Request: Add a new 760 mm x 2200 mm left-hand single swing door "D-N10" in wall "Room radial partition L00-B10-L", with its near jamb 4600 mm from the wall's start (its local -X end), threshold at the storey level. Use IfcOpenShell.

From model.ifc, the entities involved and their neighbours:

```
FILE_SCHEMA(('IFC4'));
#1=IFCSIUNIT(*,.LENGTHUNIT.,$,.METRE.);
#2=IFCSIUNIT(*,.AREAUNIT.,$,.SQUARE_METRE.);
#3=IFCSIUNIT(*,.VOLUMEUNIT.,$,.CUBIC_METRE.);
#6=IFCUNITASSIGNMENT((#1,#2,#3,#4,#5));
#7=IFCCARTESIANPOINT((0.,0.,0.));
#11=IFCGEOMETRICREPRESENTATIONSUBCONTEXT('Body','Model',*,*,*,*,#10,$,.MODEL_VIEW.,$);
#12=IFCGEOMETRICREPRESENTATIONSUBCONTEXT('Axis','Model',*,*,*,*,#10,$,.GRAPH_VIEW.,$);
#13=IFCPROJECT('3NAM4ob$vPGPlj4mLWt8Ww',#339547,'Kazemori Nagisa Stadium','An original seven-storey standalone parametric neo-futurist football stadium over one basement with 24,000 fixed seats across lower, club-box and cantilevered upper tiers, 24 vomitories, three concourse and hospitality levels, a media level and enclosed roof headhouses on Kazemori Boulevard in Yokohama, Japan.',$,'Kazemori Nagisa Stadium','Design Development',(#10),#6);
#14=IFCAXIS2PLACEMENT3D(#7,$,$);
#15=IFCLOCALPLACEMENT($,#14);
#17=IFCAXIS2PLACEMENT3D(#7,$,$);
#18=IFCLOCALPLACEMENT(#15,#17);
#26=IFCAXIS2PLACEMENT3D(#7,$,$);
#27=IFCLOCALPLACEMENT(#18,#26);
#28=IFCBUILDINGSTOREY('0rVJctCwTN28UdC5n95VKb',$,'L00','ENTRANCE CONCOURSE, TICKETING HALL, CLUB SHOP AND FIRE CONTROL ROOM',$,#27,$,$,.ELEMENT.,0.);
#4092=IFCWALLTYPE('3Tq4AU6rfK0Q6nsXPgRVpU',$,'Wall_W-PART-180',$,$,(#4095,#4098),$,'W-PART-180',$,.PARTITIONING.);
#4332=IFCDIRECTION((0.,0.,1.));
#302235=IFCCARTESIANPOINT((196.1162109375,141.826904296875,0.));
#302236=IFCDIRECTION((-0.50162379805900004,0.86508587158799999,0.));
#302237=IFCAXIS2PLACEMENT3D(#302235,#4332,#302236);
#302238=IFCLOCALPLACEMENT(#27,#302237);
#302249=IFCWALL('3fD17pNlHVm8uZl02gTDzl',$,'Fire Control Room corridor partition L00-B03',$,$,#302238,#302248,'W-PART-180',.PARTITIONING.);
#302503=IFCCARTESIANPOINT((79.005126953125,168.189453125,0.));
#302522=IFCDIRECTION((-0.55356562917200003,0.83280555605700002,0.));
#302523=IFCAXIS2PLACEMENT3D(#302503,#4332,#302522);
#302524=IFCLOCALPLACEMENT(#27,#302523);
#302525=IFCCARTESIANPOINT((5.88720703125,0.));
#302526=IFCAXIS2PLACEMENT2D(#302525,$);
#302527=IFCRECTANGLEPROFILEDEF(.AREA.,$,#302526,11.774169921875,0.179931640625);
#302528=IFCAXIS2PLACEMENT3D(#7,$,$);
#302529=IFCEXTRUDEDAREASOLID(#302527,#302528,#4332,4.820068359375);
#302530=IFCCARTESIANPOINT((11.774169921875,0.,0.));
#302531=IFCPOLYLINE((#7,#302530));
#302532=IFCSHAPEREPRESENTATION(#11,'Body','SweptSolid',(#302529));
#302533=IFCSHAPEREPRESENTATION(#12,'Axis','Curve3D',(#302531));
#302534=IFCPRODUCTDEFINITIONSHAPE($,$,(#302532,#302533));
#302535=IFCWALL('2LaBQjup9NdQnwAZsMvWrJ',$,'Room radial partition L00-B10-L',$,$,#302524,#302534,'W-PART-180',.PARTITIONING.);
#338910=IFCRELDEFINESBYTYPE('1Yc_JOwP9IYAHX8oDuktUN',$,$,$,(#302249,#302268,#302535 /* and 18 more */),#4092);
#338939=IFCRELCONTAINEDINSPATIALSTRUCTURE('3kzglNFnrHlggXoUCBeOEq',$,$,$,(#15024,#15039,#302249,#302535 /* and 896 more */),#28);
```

```python
import numpy as np
import ifcopenshell
import ifcopenshell.api.feature
import ifcopenshell.api.geometry
import ifcopenshell.api.root
import ifcopenshell.api.spatial
import ifcopenshell.geom
import ifcopenshell.util.element
import ifcopenshell.util.placement
import ifcopenshell.util.representation
import ifcopenshell.util.shape
import ifcopenshell.util.unit

model = ifcopenshell.open("model.ifc")
unit_scale = ifcopenshell.util.unit.calculate_unit_scale(model)
settings = ifcopenshell.geom.settings()


def volume(element):
    """Net volume in cubic metres, openings subtracted."""
    shape = ifcopenshell.geom.create_shape(settings, element)
    return ifcopenshell.util.shape.get_volume(shape.geometry)


wall = model.by_guid("2LaBQjup9NdQnwAZsMvWrJ")
storey = ifcopenshell.util.element.get_container(wall, ifc_class="IfcBuildingStorey")
context = ifcopenshell.util.representation.get_context(model, "Model", "Body", "MODEL_VIEW")
before = volume(wall)

width, height, from_end, sill = 0.76, 2.2, 4.6, 0.0  # metres

# The wall runs along its own X axis, and the end named is its -X end.
wall_shape = ifcopenshell.geom.create_shape(settings, wall)
x, y, z = ifcopenshell.util.shape.get_vertices(wall_shape.geometry).T
start = x.min() + from_end
face, thickness = float(y.min()), float(y.max() - y.min())
wall_matrix = ifcopenshell.util.placement.get_local_placement(wall.ObjectPlacement)
level = ifcopenshell.util.placement.get_local_placement(storey.ObjectPlacement)[2, 3]


def in_wall(x, y):
    """Placement at x, y metres in the wall's axes, at sill height."""
    matrix = wall_matrix.copy()
    matrix[:, 3] = wall_matrix @ np.array([x / unit_scale, y / unit_scale, 0.0, 1.0])
    matrix[2, 3] = level + sill / unit_scale
    return matrix


# Opening: a box that overshoots both wall faces by 50 mm.
opening = ifcopenshell.api.root.create_entity(model, ifc_class="IfcOpeningElement", predefined_type="OPENING")
box = ifcopenshell.api.geometry.add_wall_representation(
    model, context=context, length=width, height=height, thickness=thickness + 0.1
)
ifcopenshell.api.geometry.assign_representation(model, product=opening, representation=box)
ifcopenshell.api.geometry.edit_object_placement(model, product=opening, matrix=in_wall(start, face - 0.05), is_si=False)
ifcopenshell.api.feature.add_feature(model, feature=opening, element=wall)

door = ifcopenshell.api.root.create_entity(model, ifc_class="IfcDoor", name="D-N10", predefined_type="DOOR")
door.OverallWidth, door.OverallHeight = width / unit_scale, height / unit_scale
door.OperationType = "SINGLE_SWING_LEFT"
body = ifcopenshell.api.geometry.add_door_representation(
    model,
    context=context,
    overall_width=door.OverallWidth,
    overall_height=door.OverallHeight,
    operation_type="SINGLE_SWING_LEFT",
    lining_properties={"LiningDepth": thickness / unit_scale, "ThresholdDepth": thickness / unit_scale},
)
ifcopenshell.api.geometry.assign_representation(model, product=door, representation=body)
ifcopenshell.api.spatial.assign_container(model, products=[door], relating_structure=storey)
ifcopenshell.api.feature.add_filling(model, opening=opening, element=door)

# The lining spans the wall, so the door starts at the wall face.
ifcopenshell.api.geometry.edit_object_placement(model, product=door, matrix=in_wall(start, face), is_si=False)

after = volume(wall)

print(f"wall volume {before:.3f} -> {after:.3f} m3")

model.write("model_rev.ifc")
```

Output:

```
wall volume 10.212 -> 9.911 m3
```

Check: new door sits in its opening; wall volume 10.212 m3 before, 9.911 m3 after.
